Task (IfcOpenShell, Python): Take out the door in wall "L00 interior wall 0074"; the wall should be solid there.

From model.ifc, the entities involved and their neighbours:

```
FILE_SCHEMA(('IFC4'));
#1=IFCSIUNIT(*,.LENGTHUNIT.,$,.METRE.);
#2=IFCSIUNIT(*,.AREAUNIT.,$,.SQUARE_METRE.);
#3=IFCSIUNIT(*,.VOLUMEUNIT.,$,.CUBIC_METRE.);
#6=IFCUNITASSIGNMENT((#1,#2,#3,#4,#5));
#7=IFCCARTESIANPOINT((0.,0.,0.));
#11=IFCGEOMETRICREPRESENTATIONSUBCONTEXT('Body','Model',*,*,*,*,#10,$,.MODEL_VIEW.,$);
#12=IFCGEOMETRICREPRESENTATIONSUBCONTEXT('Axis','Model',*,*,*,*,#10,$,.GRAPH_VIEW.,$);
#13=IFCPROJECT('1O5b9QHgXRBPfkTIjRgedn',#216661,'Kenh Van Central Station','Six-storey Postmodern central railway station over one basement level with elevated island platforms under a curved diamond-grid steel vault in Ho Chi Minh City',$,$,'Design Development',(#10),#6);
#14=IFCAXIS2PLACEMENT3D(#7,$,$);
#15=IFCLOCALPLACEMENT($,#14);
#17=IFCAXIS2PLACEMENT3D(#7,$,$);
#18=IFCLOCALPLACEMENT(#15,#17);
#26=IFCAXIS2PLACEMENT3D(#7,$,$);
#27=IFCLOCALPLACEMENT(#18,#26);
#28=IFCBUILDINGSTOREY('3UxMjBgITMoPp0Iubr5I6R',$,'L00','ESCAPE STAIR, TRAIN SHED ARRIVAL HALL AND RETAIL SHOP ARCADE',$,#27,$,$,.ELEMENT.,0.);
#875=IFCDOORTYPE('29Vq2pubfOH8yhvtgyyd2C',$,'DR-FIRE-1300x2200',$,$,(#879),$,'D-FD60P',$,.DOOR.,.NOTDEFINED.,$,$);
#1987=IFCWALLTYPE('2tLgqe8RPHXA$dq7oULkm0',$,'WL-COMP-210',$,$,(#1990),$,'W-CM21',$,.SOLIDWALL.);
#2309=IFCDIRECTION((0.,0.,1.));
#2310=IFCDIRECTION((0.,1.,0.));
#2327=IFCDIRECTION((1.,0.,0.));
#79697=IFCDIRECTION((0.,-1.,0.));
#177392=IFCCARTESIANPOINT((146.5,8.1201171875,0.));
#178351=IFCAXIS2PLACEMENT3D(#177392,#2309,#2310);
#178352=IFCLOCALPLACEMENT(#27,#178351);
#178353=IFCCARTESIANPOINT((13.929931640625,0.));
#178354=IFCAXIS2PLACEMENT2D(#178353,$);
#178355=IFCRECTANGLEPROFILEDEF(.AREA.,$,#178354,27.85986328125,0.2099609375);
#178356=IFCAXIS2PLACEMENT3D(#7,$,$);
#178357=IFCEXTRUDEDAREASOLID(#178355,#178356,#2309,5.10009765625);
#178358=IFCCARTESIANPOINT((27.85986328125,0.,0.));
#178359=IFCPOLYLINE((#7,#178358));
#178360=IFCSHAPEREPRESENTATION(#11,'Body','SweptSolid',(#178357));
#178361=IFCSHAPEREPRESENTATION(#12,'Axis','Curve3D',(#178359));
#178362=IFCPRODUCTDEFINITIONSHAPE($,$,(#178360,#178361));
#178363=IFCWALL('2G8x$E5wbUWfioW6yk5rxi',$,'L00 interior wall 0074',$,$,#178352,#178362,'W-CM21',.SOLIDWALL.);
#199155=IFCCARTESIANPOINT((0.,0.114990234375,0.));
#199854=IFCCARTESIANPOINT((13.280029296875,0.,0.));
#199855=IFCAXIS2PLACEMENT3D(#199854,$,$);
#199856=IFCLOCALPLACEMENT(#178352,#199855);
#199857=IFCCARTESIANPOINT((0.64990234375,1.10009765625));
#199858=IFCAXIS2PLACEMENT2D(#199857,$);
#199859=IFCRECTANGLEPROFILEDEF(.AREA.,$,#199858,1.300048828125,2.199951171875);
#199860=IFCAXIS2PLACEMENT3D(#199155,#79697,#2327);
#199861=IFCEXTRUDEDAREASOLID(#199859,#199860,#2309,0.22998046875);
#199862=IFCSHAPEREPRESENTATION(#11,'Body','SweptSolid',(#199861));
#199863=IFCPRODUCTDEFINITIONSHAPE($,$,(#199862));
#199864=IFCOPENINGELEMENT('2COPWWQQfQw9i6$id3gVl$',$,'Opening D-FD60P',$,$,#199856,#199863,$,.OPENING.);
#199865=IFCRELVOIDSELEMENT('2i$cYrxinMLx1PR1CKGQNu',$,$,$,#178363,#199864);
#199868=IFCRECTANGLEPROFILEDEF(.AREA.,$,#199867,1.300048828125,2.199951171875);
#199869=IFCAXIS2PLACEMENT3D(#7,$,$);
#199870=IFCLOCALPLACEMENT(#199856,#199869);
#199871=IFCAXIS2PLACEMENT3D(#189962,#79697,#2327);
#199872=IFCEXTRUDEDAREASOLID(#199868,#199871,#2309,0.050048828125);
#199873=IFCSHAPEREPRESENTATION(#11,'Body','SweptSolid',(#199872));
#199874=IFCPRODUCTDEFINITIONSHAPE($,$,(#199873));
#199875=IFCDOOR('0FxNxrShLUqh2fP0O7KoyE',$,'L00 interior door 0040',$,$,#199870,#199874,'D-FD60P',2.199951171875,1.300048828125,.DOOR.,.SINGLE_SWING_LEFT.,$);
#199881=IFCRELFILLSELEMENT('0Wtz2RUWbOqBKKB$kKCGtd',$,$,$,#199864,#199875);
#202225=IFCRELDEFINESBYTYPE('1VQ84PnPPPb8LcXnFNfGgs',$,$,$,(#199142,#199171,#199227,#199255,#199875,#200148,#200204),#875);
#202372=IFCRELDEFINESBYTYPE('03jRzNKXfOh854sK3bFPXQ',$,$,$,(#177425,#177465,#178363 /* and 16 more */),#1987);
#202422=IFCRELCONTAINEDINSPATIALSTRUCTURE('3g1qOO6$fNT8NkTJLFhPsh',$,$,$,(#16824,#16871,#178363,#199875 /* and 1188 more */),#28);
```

```python
import ifcopenshell
import ifcopenshell.api.feature
import ifcopenshell.api.root
import ifcopenshell.geom
import ifcopenshell.util.shape

model = ifcopenshell.open("model.ifc")
settings = ifcopenshell.geom.settings()


def volume(element):
    """Net volume in cubic metres, openings subtracted."""
    shape = ifcopenshell.geom.create_shape(settings, element)
    return ifcopenshell.util.shape.get_volume(shape.geometry)


door = model.by_guid("0FxNxrShLUqh2fP0O7KoyE")
opening = door.FillsVoids[0].RelatingOpeningElement
wall = opening.VoidsElements[0].RelatingBuildingElement
before = volume(wall)

ifcopenshell.api.root.remove_product(model, product=door)
ifcopenshell.api.feature.remove_feature(model, feature=opening)

after = volume(wall)

print(f"wall volume {before:.3f} -> {after:.3f} m3")

model.write("model-out.ifc")
```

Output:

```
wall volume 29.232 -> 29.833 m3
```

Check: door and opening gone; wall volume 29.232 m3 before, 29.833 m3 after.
